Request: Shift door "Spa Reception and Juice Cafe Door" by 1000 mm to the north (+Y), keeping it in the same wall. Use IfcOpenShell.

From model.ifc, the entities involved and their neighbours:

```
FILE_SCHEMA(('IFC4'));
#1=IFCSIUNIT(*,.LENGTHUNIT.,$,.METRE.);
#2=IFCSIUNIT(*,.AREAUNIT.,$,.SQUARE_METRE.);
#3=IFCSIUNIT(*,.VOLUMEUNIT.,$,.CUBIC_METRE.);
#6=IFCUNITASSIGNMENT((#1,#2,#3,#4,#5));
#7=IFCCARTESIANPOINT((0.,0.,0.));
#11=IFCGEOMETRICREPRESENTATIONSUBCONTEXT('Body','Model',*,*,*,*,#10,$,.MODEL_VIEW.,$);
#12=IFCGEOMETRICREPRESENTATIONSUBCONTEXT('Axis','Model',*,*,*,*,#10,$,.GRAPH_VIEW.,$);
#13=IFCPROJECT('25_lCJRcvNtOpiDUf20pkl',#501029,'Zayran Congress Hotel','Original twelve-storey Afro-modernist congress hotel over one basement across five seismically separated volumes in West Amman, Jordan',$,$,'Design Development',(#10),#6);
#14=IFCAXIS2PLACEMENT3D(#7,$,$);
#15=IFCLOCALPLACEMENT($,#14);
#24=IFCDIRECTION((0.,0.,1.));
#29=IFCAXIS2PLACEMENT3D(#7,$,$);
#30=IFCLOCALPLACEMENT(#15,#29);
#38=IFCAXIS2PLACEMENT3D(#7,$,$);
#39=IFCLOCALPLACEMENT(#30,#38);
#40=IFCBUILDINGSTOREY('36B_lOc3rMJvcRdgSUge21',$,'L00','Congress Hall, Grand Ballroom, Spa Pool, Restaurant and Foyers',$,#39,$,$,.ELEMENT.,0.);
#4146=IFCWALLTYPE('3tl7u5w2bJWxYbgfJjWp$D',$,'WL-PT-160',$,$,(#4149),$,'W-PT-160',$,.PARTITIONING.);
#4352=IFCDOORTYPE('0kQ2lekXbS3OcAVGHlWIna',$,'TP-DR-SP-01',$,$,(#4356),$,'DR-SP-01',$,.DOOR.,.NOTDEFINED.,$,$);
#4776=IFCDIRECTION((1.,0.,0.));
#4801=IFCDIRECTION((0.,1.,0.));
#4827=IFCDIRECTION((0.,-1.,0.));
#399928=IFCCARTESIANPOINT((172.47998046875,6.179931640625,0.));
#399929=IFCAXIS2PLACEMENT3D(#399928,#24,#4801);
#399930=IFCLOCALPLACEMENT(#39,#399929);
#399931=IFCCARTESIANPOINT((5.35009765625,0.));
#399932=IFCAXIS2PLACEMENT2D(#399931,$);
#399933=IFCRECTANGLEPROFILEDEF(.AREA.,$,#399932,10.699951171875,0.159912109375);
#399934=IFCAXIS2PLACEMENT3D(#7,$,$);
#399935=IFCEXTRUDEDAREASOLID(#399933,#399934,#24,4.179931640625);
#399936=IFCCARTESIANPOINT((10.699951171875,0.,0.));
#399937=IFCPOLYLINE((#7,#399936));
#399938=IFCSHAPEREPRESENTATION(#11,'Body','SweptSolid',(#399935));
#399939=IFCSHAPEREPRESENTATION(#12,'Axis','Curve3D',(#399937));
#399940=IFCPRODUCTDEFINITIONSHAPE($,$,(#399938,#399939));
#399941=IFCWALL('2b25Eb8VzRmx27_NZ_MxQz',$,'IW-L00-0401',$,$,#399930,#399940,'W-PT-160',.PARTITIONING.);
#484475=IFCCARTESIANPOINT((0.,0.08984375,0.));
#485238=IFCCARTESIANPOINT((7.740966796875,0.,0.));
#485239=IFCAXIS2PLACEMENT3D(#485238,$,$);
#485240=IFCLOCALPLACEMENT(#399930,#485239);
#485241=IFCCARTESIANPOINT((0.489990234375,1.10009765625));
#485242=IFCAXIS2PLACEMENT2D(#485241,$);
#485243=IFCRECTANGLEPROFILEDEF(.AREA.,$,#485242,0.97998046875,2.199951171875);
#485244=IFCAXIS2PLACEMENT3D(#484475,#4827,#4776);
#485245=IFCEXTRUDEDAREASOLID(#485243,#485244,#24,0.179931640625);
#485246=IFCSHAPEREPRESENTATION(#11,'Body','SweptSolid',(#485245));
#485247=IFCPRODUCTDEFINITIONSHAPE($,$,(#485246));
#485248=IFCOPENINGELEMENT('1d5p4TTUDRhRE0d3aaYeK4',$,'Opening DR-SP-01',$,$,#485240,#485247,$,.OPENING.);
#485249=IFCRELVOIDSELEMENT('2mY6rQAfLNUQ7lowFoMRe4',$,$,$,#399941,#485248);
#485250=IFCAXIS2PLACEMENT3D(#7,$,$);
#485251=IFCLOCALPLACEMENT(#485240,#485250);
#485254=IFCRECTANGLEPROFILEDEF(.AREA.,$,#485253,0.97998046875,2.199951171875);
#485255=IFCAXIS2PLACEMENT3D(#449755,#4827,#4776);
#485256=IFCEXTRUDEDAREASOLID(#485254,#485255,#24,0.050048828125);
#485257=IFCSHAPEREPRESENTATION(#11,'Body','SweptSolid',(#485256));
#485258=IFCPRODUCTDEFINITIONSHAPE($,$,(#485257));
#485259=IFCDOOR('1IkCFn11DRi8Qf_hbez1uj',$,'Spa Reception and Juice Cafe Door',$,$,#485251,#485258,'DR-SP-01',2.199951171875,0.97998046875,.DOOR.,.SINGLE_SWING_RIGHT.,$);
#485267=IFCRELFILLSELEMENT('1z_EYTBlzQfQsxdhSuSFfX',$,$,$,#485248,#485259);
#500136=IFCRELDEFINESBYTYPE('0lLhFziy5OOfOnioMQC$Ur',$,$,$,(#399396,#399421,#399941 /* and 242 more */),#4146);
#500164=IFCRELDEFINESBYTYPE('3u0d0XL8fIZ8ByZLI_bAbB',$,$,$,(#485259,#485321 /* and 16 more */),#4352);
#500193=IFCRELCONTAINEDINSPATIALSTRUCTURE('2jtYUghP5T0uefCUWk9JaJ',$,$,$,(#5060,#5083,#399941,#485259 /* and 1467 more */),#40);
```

```python
import ifcopenshell
import ifcopenshell.api.geometry
import ifcopenshell.util.placement
import ifcopenshell.util.unit

model = ifcopenshell.open("model.ifc")
unit_scale = ifcopenshell.util.unit.calculate_unit_scale(model)

door = model.by_guid("1IkCFn11DRi8Qf_hbez1uj")
opening = door.FillsVoids[0].RelatingOpeningElement
wall = opening.VoidsElements[0].RelatingBuildingElement

wall_matrix = ifcopenshell.util.placement.get_local_placement(wall.ObjectPlacement)
shift = wall_matrix[:3, 0] * 1 / unit_scale
before = ifcopenshell.util.placement.get_local_placement(door.ObjectPlacement)[:3, 3].copy()

# The door is placed relative to its opening, so it follows when the opening moves.
matrix = ifcopenshell.util.placement.get_local_placement(opening.ObjectPlacement)
matrix[:3, 3] += shift
ifcopenshell.api.geometry.edit_object_placement(
    model, product=opening, matrix=matrix, is_si=False, should_transform_children=True
)

after = ifcopenshell.util.placement.get_local_placement(door.ObjectPlacement)[:3, 3]
print("door moved by", (after - before).round(3) + 0.0)

model.write("model_updated.ifc")
```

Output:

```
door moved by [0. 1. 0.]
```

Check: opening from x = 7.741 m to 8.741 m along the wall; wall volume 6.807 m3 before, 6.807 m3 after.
